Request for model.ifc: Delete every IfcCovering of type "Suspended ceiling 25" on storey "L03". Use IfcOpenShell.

First a look at what the model holds.

```python
import ifcopenshell
import ifcopenshell.util.element

model = ifcopenshell.open("model.ifc")
print(model.schema)
storey = next(s for s in model.by_type("IfcBuildingStorey") if s.Name == "L03")
coverings = [e for e in ifcopenshell.util.element.get_decomposition(storey) if e.is_a("IfcCovering")]
seen = {}
for e in coverings:
    element_type = ifcopenshell.util.element.get_type(e)
    name = element_type.Name if element_type not in (None, e) else None
    seen[name] = seen.get(name, 0) + 1
for name, count in sorted(seen.items(), key=str):
    print(count, "x", name)
```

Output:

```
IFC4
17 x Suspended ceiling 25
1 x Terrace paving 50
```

```python
import ifcopenshell
import ifcopenshell.api.root
import ifcopenshell.util.element

model = ifcopenshell.open("model.ifc")

storey = next(s for s in model.by_type("IfcBuildingStorey") if s.Name == "L03")
coverings = [e for e in ifcopenshell.util.element.get_decomposition(storey) if e.is_a("IfcCovering")]
targets = [e for e in coverings if (t := ifcopenshell.util.element.get_type(e)) not in (None, e) and t.Name == "Suspended ceiling 25"]

for e in targets:
    ifcopenshell.api.root.remove_product(model, product=e)
print(len(targets), "removed")

model.write("model_updated.ifc")
```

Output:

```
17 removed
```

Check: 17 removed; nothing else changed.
